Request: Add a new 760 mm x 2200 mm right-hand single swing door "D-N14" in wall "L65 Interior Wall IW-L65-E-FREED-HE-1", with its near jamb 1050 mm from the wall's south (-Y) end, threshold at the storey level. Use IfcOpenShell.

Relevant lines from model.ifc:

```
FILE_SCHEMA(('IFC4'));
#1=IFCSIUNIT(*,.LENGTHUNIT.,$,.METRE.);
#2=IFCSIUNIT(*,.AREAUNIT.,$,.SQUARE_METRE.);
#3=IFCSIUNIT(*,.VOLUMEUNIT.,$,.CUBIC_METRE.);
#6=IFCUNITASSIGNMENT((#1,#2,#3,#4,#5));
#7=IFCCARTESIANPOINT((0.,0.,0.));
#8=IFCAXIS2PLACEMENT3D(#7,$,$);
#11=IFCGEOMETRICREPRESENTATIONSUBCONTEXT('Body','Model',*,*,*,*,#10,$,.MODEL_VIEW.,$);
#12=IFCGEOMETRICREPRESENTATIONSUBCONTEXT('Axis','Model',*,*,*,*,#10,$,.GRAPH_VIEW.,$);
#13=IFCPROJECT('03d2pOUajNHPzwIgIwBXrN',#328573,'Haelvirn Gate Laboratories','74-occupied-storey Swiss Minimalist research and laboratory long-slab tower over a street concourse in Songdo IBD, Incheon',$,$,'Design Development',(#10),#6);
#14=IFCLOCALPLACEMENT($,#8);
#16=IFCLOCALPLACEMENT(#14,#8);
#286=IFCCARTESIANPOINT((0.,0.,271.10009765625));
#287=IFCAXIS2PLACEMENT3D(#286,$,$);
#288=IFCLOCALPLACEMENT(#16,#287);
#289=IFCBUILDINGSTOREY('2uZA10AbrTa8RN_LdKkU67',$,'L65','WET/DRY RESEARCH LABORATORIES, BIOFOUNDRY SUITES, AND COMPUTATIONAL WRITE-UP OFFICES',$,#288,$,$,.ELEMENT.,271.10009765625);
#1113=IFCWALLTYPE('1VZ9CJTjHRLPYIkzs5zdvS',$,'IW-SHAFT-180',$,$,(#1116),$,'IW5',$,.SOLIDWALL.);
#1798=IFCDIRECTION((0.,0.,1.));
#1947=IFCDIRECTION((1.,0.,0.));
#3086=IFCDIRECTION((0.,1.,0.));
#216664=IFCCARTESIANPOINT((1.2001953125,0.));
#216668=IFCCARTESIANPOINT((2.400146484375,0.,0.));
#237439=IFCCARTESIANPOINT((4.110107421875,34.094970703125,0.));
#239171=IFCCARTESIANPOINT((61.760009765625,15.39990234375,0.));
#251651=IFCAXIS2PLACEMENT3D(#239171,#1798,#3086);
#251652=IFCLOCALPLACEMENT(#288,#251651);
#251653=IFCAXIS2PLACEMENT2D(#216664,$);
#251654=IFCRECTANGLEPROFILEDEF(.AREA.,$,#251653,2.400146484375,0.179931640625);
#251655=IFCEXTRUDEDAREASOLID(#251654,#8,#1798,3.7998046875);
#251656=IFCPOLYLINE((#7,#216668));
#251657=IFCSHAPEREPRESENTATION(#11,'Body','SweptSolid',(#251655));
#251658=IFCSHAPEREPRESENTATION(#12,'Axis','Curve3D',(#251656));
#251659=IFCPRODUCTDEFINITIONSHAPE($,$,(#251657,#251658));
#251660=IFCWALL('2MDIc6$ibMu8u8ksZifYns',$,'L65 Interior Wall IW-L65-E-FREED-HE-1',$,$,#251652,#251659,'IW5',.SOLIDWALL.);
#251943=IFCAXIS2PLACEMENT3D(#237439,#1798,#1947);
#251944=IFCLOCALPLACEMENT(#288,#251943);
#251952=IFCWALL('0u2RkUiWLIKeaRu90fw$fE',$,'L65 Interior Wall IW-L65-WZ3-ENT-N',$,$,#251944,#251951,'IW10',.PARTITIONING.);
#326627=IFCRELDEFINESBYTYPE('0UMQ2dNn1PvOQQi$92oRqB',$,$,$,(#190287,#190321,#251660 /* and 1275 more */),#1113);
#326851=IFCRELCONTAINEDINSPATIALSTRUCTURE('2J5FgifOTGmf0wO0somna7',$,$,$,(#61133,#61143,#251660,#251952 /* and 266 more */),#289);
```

```python
import numpy as np
import ifcopenshell
import ifcopenshell.api.feature
import ifcopenshell.api.geometry
import ifcopenshell.api.root
import ifcopenshell.api.spatial
import ifcopenshell.geom
import ifcopenshell.util.element
import ifcopenshell.util.placement
import ifcopenshell.util.representation
import ifcopenshell.util.shape
import ifcopenshell.util.unit

model = ifcopenshell.open("model.ifc")
unit_scale = ifcopenshell.util.unit.calculate_unit_scale(model)
settings = ifcopenshell.geom.settings()


def volume(element):
    """Net volume in cubic metres, openings subtracted."""
    shape = ifcopenshell.geom.create_shape(settings, element)
    return ifcopenshell.util.shape.get_volume(shape.geometry)


wall = model.by_id(251660)
storey = ifcopenshell.util.element.get_container(wall, ifc_class="IfcBuildingStorey")
context = ifcopenshell.util.representation.get_context(model, "Model", "Body", "MODEL_VIEW")
before = volume(wall)

width, height, from_end, sill = 0.76, 2.2, 1.05, 0.0  # metres

# The wall runs along its own X axis, and the end named is its -X end.
wall_shape = ifcopenshell.geom.create_shape(settings, wall)
x, y, z = ifcopenshell.util.shape.get_vertices(wall_shape.geometry).T
start = x.min() + from_end
face, thickness = float(y.min()), float(y.max() - y.min())
wall_matrix = ifcopenshell.util.placement.get_local_placement(wall.ObjectPlacement)
level = ifcopenshell.util.placement.get_local_placement(storey.ObjectPlacement)[2, 3]


def in_wall(x, y):
    """Placement at x, y metres in the wall's axes, at sill height."""
    matrix = wall_matrix.copy()
    matrix[:, 3] = wall_matrix @ np.array([x / unit_scale, y / unit_scale, 0.0, 1.0])
    matrix[2, 3] = level + sill / unit_scale
    return matrix


# Opening: a box that overshoots both wall faces by 50 mm.
opening = ifcopenshell.api.root.create_entity(model, ifc_class="IfcOpeningElement", predefined_type="OPENING")
box = ifcopenshell.api.geometry.add_wall_representation(
    model, context=context, length=width, height=height, thickness=thickness + 0.1
)
ifcopenshell.api.geometry.assign_representation(model, product=opening, representation=box)
ifcopenshell.api.geometry.edit_object_placement(model, product=opening, matrix=in_wall(start, face - 0.05), is_si=False)
ifcopenshell.api.feature.add_feature(model, feature=opening, element=wall)

door = ifcopenshell.api.root.create_entity(model, ifc_class="IfcDoor", name="D-N14", predefined_type="DOOR")
door.OverallWidth, door.OverallHeight = width / unit_scale, height / unit_scale
door.OperationType = "SINGLE_SWING_RIGHT"
body = ifcopenshell.api.geometry.add_door_representation(
    model,
    context=context,
    overall_width=door.OverallWidth,
    overall_height=door.OverallHeight,
    operation_type="SINGLE_SWING_RIGHT",
    lining_properties={"LiningDepth": thickness / unit_scale, "ThresholdDepth": thickness / unit_scale},
)
ifcopenshell.api.geometry.assign_representation(model, product=door, representation=body)
ifcopenshell.api.spatial.assign_container(model, products=[door], relating_structure=storey)
ifcopenshell.api.feature.add_filling(model, opening=opening, element=door)

# The lining spans the wall, so the door starts at the wall face.
ifcopenshell.api.geometry.edit_object_placement(model, product=door, matrix=in_wall(start, face), is_si=False)

after = volume(wall)

print(f"wall volume {before:.3f} -> {after:.3f} m3")

model.write("model_edited.ifc")
```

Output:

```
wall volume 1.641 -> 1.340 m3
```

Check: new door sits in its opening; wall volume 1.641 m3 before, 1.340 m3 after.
